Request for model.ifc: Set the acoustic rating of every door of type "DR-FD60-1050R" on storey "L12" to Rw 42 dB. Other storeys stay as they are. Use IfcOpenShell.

First a look at what the model holds.

```python
import ifcopenshell
import ifcopenshell.util.element

model = ifcopenshell.open("model.ifc")
print(model.schema)
storey = next(s for s in model.by_type("IfcBuildingStorey") if s.Name == "L12")
doors = [e for e in ifcopenshell.util.element.get_decomposition(storey) if e.is_a("IfcDoor")]
seen = {}
for e in doors:
    element_type = ifcopenshell.util.element.get_type(e)
    key = (element_type.Name if element_type != e and element_type else None, ifcopenshell.util.element.get_pset(e, "Pset_DoorCommon", "AcousticRating"))
    seen[key] = seen.get(key, 0) + 1
for (name, value), count in sorted(seen.items(), key=str):
    print(count, "x", name, "|", value)
```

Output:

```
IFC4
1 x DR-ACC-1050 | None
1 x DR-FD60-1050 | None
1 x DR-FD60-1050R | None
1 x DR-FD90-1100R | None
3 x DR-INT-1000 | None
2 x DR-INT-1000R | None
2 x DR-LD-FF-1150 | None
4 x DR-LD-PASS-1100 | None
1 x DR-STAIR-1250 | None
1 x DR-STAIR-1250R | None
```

```python
import ifcopenshell
import ifcopenshell.api.pset
import ifcopenshell.util.element

model = ifcopenshell.open("model.ifc")

storey = next(s for s in model.by_type("IfcBuildingStorey") if s.Name == "L12")
doors = [e for e in ifcopenshell.util.element.get_decomposition(storey) if e.is_a("IfcDoor")]

count = 0
for e in doors:
    element_type = ifcopenshell.util.element.get_type(e)
    if element_type in (None, e) or element_type.Name != "DR-FD60-1050R":
        continue
    # add_pset returns the element's existing set when there is one.
    pset = ifcopenshell.api.pset.add_pset(model, product=e, name="Pset_DoorCommon")
    ifcopenshell.api.pset.edit_pset(model, pset=pset, properties={"AcousticRating": "Rw 42 dB"})
    count += 1

print(count, "doors updated")

model.write("model_rev.ifc")
```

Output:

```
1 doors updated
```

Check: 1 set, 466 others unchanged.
